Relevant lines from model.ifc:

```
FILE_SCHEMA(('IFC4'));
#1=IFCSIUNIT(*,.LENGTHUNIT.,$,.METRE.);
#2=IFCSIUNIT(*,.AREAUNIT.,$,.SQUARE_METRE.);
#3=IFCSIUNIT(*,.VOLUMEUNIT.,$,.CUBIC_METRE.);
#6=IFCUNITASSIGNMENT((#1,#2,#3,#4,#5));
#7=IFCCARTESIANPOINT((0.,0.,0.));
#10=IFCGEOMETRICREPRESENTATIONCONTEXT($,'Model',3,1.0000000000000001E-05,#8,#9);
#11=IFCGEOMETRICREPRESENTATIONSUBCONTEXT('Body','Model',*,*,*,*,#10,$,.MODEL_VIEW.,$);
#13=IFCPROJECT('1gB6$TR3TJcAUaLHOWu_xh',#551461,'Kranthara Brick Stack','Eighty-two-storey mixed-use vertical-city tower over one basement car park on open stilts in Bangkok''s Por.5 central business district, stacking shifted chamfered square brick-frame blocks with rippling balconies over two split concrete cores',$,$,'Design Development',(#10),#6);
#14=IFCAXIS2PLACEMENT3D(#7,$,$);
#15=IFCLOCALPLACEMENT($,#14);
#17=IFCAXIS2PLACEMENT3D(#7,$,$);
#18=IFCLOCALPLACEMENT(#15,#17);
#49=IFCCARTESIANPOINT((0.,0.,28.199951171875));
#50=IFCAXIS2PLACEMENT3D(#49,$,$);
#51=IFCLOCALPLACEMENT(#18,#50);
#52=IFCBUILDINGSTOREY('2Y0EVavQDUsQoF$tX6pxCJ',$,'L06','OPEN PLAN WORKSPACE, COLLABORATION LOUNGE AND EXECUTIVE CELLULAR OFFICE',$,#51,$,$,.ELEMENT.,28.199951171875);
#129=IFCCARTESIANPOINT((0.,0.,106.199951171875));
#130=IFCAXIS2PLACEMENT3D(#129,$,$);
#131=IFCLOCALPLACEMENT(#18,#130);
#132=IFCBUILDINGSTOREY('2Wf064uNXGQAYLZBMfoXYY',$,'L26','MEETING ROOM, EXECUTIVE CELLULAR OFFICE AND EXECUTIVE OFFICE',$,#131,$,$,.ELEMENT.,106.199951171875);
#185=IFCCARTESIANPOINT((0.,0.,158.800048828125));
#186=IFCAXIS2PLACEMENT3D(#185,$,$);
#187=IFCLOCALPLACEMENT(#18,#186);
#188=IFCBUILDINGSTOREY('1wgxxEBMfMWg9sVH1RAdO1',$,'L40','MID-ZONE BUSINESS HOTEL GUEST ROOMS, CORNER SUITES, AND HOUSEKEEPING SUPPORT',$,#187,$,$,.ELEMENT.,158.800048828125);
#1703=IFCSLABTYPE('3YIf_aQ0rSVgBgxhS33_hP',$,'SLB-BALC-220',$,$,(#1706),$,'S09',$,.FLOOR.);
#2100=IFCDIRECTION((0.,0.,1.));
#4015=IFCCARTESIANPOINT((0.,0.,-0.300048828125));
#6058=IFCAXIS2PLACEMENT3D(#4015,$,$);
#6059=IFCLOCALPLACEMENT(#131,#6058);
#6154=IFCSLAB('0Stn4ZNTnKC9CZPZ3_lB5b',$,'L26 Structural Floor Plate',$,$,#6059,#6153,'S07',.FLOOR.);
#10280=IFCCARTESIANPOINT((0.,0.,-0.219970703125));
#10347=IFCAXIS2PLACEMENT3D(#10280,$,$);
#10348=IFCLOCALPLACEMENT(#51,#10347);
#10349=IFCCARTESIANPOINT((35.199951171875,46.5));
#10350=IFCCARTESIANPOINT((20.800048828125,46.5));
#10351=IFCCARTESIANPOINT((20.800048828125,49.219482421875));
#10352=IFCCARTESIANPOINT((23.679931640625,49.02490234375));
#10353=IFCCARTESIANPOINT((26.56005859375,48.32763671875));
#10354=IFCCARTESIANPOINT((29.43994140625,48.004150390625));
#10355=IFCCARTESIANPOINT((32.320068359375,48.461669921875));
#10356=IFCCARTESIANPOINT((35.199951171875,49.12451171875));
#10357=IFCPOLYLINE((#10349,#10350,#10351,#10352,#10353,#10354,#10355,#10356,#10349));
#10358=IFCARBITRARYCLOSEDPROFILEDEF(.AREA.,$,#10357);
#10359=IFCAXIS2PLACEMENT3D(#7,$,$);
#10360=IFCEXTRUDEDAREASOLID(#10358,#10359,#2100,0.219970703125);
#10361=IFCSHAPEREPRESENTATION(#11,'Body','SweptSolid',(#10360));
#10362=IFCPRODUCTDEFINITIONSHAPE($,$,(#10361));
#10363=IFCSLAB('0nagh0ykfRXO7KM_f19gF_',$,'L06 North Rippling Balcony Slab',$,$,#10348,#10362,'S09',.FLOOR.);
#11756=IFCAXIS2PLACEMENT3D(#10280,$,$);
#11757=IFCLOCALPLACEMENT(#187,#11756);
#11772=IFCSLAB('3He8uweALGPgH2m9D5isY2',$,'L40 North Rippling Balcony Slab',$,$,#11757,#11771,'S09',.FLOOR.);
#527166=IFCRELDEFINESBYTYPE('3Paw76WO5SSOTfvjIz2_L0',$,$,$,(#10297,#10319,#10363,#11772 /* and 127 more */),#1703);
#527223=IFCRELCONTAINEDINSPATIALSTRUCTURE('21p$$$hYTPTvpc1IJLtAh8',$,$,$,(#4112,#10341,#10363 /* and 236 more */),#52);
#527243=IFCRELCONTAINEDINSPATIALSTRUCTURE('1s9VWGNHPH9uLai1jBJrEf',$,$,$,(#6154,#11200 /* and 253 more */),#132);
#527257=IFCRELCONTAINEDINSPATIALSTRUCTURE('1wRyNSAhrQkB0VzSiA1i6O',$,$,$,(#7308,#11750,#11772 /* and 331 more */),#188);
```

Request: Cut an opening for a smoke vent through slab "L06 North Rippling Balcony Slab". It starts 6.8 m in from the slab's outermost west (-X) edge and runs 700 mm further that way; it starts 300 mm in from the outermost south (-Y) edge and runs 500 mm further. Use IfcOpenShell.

```python
import numpy as np
import ifcopenshell
import ifcopenshell.api.feature
import ifcopenshell.api.geometry
import ifcopenshell.api.root
import ifcopenshell.geom
import ifcopenshell.util.placement
import ifcopenshell.util.representation
import ifcopenshell.util.shape
import ifcopenshell.util.unit

model = ifcopenshell.open("model.ifc")
unit_scale = ifcopenshell.util.unit.calculate_unit_scale(model)
settings = ifcopenshell.geom.settings()


def volume(element):
    """Net volume in cubic metres, openings subtracted."""
    shape = ifcopenshell.geom.create_shape(settings, element)
    return ifcopenshell.util.shape.get_volume(shape.geometry)


slab = model.by_id(10363)
before = volume(slab)

# Extent in the slab's own axes, in metres. The edges named are its -X and -Y sides.
slab_shape = ifcopenshell.geom.create_shape(settings, slab)
vertices = ifcopenshell.util.shape.get_vertices(slab_shape.geometry)
x_min, y_min, bottom = vertices.min(axis=0)
top = vertices[:, 2].max()

opening = ifcopenshell.api.root.create_entity(model, ifc_class="IfcOpeningElement", name="Smoke vent opening", predefined_type="OPENING")
context = ifcopenshell.util.representation.get_context(model, "Model", "Body", "MODEL_VIEW")
width, depth = 0.7, 0.5
outline = [(0.0, 0.0), (width, 0.0), (width, depth), (0.0, depth), (0.0, 0.0)]
# Overshoot both faces by 50 mm so the cut is clean.
shape = ifcopenshell.api.geometry.add_slab_representation(
    model, context=context, depth=top - bottom + 0.1, polyline=outline
)
ifcopenshell.api.geometry.assign_representation(model, product=opening, representation=shape)

matrix = ifcopenshell.util.placement.get_local_placement(slab.ObjectPlacement)
matrix[:, 3] = matrix @ np.append(np.array([x_min + 6.8, y_min + 0.3, bottom - 0.05]) / unit_scale, 1.0)
ifcopenshell.api.geometry.edit_object_placement(model, product=opening, matrix=matrix, is_si=False)
ifcopenshell.api.feature.add_feature(model, feature=opening, element=slab)

after = volume(slab)

print(f"slab volume {before:.3f} -> {after:.3f} m3")

model.write("model-out.ifc")
```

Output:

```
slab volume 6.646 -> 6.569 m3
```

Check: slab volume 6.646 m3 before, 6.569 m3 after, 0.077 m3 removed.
